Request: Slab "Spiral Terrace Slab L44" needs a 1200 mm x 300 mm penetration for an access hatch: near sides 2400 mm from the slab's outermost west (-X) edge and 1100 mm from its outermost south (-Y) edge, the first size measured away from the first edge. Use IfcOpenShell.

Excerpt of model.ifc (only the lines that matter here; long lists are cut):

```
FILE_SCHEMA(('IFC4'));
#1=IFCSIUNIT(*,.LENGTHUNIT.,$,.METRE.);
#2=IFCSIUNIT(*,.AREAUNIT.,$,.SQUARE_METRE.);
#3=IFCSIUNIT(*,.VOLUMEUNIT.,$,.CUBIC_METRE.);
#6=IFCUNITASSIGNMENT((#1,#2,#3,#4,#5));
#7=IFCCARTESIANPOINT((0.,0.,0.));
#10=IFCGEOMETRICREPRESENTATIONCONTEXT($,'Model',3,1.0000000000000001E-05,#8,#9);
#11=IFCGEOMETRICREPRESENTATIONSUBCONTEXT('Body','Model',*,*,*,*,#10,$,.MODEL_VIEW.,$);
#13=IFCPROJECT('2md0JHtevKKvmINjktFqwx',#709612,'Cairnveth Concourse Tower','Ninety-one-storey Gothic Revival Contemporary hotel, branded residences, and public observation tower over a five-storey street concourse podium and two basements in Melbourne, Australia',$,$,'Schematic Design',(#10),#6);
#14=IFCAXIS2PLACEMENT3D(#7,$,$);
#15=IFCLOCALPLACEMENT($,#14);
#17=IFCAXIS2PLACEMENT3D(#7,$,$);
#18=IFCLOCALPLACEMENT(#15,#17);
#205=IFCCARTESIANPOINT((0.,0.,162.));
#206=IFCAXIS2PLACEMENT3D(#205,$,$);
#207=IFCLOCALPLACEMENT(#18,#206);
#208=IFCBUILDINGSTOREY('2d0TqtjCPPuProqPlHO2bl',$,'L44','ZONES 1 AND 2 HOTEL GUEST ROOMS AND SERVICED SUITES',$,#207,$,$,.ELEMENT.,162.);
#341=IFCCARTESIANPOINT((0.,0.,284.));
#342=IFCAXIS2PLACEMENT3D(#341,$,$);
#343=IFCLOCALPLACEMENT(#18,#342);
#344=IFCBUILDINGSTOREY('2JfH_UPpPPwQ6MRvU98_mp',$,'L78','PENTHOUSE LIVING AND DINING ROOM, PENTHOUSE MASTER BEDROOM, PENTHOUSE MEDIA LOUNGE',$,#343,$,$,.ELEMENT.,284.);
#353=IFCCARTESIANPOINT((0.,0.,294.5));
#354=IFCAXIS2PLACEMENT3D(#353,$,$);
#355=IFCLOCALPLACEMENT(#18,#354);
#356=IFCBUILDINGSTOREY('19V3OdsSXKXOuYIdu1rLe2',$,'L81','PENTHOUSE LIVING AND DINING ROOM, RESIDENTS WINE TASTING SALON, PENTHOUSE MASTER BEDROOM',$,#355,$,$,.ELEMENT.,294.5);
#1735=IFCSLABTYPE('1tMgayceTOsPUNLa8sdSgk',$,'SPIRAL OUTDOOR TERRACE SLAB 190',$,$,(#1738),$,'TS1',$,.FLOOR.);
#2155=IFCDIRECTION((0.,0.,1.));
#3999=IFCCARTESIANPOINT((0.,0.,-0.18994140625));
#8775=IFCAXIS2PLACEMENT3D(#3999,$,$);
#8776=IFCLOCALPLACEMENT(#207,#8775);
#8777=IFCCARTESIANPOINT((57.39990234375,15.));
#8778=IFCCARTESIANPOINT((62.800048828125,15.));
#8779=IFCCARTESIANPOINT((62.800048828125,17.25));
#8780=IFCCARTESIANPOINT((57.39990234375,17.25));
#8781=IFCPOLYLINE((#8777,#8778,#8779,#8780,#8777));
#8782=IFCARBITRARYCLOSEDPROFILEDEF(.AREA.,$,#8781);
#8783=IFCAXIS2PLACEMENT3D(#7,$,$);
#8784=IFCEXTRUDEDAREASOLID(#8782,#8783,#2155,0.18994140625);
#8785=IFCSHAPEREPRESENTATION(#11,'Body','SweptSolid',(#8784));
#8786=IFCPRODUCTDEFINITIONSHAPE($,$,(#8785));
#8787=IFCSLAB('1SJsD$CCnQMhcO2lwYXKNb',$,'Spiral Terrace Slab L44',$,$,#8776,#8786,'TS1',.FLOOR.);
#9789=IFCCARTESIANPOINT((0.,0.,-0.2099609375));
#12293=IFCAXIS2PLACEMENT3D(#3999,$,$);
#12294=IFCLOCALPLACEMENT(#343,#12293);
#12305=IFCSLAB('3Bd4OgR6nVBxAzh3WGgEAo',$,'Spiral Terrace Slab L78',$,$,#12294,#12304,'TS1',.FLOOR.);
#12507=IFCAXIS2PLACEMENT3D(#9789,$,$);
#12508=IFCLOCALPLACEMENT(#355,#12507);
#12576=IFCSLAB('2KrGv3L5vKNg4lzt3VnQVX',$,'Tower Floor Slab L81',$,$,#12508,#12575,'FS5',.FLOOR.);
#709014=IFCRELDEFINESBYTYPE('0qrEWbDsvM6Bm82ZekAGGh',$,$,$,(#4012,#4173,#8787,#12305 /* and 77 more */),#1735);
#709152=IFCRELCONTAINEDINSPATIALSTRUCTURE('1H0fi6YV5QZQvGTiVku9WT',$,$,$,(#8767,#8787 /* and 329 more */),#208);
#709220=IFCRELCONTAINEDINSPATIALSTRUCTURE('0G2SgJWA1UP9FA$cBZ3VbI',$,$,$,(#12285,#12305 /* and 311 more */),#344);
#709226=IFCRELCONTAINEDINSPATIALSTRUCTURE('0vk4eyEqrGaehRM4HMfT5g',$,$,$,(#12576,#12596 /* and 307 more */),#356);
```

```python
import numpy as np
import ifcopenshell
import ifcopenshell.api.feature
import ifcopenshell.api.geometry
import ifcopenshell.api.root
import ifcopenshell.geom
import ifcopenshell.util.placement
import ifcopenshell.util.representation
import ifcopenshell.util.shape
import ifcopenshell.util.unit

model = ifcopenshell.open("model.ifc")
unit_scale = ifcopenshell.util.unit.calculate_unit_scale(model)
settings = ifcopenshell.geom.settings()


def volume(element):
    """Net volume in cubic metres, openings subtracted."""
    shape = ifcopenshell.geom.create_shape(settings, element)
    return ifcopenshell.util.shape.get_volume(shape.geometry)


slab = model.by_guid("1SJsD$CCnQMhcO2lwYXKNb")
before = volume(slab)

# Extent in the slab's own axes, in metres. The edges named are its -X and -Y sides.
slab_shape = ifcopenshell.geom.create_shape(settings, slab)
vertices = ifcopenshell.util.shape.get_vertices(slab_shape.geometry)
x_min, y_min, bottom = vertices.min(axis=0)
top = vertices[:, 2].max()

opening = ifcopenshell.api.root.create_entity(model, ifc_class="IfcOpeningElement", name="Access hatch opening", predefined_type="OPENING")
context = ifcopenshell.util.representation.get_context(model, "Model", "Body", "MODEL_VIEW")
width, depth = 1.2, 0.3
outline = [(0.0, 0.0), (width, 0.0), (width, depth), (0.0, depth), (0.0, 0.0)]
# Overshoot both faces by 50 mm so the cut is clean.
shape = ifcopenshell.api.geometry.add_slab_representation(
    model, context=context, depth=top - bottom + 0.1, polyline=outline
)
ifcopenshell.api.geometry.assign_representation(model, product=opening, representation=shape)

matrix = ifcopenshell.util.placement.get_local_placement(slab.ObjectPlacement)
matrix[:, 3] = matrix @ np.append(np.array([x_min + 2.4, y_min + 1.1, bottom - 0.05]) / unit_scale, 1.0)
ifcopenshell.api.geometry.edit_object_placement(model, product=opening, matrix=matrix, is_si=False)
ifcopenshell.api.feature.add_feature(model, feature=opening, element=slab)

after = volume(slab)

print(f"slab volume {before:.3f} -> {after:.3f} m3")

model.write("model_rev.ifc")
```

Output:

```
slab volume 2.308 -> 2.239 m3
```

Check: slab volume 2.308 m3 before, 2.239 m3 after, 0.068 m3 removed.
